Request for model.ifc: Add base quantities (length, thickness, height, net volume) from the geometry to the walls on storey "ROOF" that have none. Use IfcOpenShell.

First a look at what the model holds.

```python
import ifcopenshell
import ifcopenshell.util.element
import ifcopenshell.util.unit

model = ifcopenshell.open("model.ifc")
print(model.schema)
for unit_type in ("LENGTHUNIT", "AREAUNIT", "VOLUMEUNIT"):
    print(unit_type, ifcopenshell.util.unit.calculate_unit_scale(model, unit_type))
storey = next(s for s in model.by_type("IfcBuildingStorey") if s.Name == "ROOF")
walls = [e for e in ifcopenshell.util.element.get_decomposition(storey) if e.is_a("IfcWall")]
for e in sorted(walls, key=lambda e: e.id()):
    print(e.id(), e.is_a(), e.Name, list(ifcopenshell.util.element.get_psets(e, qtos_only=True)), sep=" | ")
```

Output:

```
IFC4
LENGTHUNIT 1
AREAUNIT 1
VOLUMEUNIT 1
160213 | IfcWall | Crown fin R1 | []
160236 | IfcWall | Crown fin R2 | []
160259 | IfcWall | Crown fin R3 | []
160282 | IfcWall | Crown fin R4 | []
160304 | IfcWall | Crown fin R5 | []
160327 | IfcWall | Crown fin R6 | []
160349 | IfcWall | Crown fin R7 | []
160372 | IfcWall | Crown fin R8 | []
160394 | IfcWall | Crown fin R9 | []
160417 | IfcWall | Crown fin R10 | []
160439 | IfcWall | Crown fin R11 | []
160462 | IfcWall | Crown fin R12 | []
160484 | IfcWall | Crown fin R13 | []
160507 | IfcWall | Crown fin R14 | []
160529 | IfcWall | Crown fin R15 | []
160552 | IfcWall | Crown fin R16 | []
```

```python
import ifcopenshell
import ifcopenshell.api.pset
import ifcopenshell.geom
import ifcopenshell.util.element
import ifcopenshell.util.shape
import ifcopenshell.util.unit

model = ifcopenshell.open("model.ifc")
unit_scale = ifcopenshell.util.unit.calculate_unit_scale(model)
volume_scale = ifcopenshell.util.unit.calculate_unit_scale(model, "VOLUMEUNIT")
settings = ifcopenshell.geom.settings()

storey = next(s for s in model.by_type("IfcBuildingStorey") if s.Name == "ROOF")
walls = [e for e in ifcopenshell.util.element.get_decomposition(storey) if e.is_a("IfcWall")]

for e in sorted(walls, key=lambda e: e.id()):
    if ifcopenshell.util.element.get_psets(e, qtos_only=True, should_inherit=False):
        continue
    # Geometry comes back in metres, in the element's own axes.
    shape = ifcopenshell.geom.create_shape(settings, e)
    values = {
        "Length": ifcopenshell.util.shape.get_x(shape.geometry) / unit_scale,
        "Width": ifcopenshell.util.shape.get_y(shape.geometry) / unit_scale,
        "Height": ifcopenshell.util.shape.get_z(shape.geometry) / unit_scale,
        "NetVolume": ifcopenshell.util.shape.get_volume(shape.geometry) / volume_scale,
    }
    qto = ifcopenshell.api.pset.add_qto(model, product=e, name="Qto_WallBaseQuantities")
    ifcopenshell.api.pset.edit_qto(model, qto=qto, properties=values)
    print(e.id(), {k: round(v, 3) for k, v in values.items()})

model.write("model_updated.ifc")
```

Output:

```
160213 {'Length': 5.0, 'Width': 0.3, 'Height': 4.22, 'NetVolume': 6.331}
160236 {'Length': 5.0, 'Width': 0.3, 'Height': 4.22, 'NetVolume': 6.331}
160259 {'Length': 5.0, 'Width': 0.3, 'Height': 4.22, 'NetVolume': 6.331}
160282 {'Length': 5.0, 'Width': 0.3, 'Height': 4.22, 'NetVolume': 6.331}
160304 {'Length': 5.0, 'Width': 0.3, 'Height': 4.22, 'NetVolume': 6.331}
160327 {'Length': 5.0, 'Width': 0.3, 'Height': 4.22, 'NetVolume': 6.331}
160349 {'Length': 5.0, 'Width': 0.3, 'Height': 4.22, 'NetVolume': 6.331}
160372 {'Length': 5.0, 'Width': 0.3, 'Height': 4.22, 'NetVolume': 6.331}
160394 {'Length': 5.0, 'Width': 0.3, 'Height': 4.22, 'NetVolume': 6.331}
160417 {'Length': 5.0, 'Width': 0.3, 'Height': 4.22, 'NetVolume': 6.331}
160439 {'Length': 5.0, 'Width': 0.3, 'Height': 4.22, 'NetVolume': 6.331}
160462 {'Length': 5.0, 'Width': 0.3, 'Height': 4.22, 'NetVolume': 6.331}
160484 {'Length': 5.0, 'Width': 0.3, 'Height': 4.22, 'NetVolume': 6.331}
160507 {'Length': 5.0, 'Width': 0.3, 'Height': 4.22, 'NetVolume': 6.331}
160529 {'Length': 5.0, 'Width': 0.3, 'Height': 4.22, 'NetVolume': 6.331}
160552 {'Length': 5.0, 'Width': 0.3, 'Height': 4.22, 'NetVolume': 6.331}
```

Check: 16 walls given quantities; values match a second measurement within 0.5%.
